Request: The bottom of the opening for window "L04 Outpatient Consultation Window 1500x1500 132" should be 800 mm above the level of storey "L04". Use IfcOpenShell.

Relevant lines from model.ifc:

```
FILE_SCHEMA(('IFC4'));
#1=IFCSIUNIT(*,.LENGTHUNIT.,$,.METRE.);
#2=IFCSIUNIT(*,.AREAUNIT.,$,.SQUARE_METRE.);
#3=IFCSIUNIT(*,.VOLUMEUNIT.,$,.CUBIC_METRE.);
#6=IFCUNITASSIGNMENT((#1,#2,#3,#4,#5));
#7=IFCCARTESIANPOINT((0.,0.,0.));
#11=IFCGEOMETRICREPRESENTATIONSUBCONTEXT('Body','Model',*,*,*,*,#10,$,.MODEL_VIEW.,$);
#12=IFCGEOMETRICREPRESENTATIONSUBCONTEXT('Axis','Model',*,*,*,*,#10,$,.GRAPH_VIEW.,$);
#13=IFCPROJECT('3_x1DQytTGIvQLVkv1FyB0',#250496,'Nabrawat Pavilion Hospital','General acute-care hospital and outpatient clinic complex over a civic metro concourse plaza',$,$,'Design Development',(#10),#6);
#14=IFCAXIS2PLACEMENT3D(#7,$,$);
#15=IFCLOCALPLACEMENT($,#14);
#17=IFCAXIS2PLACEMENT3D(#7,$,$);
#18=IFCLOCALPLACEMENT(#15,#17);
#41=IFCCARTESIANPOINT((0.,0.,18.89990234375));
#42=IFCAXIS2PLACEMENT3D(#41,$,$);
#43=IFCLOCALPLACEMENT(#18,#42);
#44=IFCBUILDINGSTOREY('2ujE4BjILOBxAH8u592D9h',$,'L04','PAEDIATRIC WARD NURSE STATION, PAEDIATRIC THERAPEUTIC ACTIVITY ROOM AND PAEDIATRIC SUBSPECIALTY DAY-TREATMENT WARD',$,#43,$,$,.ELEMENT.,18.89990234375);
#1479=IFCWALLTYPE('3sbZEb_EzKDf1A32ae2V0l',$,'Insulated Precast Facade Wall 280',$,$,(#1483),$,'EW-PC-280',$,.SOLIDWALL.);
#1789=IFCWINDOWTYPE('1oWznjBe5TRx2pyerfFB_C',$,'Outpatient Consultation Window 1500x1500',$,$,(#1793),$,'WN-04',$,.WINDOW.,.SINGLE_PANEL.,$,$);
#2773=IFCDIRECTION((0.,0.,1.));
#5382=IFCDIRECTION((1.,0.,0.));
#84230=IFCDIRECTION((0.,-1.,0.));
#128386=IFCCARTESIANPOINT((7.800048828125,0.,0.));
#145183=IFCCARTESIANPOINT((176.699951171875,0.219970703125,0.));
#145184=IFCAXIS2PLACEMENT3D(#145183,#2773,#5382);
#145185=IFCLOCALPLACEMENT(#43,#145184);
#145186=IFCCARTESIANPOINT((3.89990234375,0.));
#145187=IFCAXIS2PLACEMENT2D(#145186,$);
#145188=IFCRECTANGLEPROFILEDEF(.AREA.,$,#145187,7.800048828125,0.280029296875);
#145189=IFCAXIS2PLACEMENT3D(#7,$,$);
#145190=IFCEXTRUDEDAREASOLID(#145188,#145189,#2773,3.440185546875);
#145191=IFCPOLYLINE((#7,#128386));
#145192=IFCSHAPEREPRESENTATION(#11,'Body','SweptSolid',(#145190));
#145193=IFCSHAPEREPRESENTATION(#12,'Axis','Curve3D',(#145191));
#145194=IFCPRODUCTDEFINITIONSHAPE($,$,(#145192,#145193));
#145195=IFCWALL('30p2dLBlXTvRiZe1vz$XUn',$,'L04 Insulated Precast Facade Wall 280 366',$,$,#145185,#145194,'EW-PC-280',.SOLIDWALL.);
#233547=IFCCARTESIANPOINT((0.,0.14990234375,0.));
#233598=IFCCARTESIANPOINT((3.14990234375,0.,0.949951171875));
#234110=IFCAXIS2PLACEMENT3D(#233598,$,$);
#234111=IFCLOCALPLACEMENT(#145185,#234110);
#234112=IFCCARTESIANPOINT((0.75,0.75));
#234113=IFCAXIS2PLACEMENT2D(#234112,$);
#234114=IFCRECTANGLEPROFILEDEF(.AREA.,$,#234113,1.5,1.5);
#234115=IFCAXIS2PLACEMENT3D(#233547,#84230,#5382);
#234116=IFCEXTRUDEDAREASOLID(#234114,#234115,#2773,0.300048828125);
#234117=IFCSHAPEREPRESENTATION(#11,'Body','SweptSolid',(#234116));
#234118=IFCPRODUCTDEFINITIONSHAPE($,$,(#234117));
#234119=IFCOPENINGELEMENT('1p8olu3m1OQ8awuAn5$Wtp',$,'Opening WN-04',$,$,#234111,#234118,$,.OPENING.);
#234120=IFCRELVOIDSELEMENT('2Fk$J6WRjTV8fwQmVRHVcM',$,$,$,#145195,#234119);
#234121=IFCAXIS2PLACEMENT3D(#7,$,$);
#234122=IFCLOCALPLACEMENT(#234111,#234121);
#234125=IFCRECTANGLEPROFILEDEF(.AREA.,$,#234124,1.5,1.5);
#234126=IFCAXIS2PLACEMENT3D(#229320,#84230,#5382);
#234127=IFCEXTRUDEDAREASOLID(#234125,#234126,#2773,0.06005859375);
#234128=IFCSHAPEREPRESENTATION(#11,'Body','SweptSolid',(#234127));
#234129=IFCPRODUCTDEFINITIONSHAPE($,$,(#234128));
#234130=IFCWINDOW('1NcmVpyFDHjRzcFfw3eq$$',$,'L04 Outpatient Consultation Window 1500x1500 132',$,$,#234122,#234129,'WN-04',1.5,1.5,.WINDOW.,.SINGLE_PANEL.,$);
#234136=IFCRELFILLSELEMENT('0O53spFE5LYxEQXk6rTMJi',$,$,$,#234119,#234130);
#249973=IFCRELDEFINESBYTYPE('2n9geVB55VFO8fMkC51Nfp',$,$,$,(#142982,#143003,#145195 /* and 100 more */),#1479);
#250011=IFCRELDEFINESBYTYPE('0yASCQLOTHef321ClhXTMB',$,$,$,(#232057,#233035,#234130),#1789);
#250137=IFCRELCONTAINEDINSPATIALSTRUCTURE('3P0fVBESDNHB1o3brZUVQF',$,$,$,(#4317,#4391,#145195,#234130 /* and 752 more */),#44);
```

```python
import numpy as np
import ifcopenshell
import ifcopenshell.api.geometry
import ifcopenshell.geom
import ifcopenshell.util.element
import ifcopenshell.util.placement
import ifcopenshell.util.shape
import ifcopenshell.util.unit

model = ifcopenshell.open("model.ifc")
unit_scale = ifcopenshell.util.unit.calculate_unit_scale(model)

window = model.by_guid("1NcmVpyFDHjRzcFfw3eq$$")
opening = window.FillsVoids[0].RelatingOpeningElement
storey = ifcopenshell.util.element.get_container(window, ifc_class="IfcBuildingStorey")
level = ifcopenshell.util.placement.get_local_placement(storey.ObjectPlacement)[2, 3]

# The opening's origin need not be at the sill, so measure its lowest point.
shape = ifcopenshell.geom.create_shape(ifcopenshell.geom.settings(), opening)
bottom = ifcopenshell.util.shape.get_shape_bottom_elevation(shape, shape.geometry) / unit_scale
dz = level + 0.8 / unit_scale - bottom

shift = np.array([0.0, 0.0, dz])
# The window is placed relative to its opening, so it follows when the opening moves.
matrix = ifcopenshell.util.placement.get_local_placement(opening.ObjectPlacement)
matrix[:3, 3] += shift
ifcopenshell.api.geometry.edit_object_placement(
    model, product=opening, matrix=matrix, is_si=False, should_transform_children=True
)

print(f"moved by {dz * unit_scale:+.3f} m")

model.write("model_v2.ifc")
```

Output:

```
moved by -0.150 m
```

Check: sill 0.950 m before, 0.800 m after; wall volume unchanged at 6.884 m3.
